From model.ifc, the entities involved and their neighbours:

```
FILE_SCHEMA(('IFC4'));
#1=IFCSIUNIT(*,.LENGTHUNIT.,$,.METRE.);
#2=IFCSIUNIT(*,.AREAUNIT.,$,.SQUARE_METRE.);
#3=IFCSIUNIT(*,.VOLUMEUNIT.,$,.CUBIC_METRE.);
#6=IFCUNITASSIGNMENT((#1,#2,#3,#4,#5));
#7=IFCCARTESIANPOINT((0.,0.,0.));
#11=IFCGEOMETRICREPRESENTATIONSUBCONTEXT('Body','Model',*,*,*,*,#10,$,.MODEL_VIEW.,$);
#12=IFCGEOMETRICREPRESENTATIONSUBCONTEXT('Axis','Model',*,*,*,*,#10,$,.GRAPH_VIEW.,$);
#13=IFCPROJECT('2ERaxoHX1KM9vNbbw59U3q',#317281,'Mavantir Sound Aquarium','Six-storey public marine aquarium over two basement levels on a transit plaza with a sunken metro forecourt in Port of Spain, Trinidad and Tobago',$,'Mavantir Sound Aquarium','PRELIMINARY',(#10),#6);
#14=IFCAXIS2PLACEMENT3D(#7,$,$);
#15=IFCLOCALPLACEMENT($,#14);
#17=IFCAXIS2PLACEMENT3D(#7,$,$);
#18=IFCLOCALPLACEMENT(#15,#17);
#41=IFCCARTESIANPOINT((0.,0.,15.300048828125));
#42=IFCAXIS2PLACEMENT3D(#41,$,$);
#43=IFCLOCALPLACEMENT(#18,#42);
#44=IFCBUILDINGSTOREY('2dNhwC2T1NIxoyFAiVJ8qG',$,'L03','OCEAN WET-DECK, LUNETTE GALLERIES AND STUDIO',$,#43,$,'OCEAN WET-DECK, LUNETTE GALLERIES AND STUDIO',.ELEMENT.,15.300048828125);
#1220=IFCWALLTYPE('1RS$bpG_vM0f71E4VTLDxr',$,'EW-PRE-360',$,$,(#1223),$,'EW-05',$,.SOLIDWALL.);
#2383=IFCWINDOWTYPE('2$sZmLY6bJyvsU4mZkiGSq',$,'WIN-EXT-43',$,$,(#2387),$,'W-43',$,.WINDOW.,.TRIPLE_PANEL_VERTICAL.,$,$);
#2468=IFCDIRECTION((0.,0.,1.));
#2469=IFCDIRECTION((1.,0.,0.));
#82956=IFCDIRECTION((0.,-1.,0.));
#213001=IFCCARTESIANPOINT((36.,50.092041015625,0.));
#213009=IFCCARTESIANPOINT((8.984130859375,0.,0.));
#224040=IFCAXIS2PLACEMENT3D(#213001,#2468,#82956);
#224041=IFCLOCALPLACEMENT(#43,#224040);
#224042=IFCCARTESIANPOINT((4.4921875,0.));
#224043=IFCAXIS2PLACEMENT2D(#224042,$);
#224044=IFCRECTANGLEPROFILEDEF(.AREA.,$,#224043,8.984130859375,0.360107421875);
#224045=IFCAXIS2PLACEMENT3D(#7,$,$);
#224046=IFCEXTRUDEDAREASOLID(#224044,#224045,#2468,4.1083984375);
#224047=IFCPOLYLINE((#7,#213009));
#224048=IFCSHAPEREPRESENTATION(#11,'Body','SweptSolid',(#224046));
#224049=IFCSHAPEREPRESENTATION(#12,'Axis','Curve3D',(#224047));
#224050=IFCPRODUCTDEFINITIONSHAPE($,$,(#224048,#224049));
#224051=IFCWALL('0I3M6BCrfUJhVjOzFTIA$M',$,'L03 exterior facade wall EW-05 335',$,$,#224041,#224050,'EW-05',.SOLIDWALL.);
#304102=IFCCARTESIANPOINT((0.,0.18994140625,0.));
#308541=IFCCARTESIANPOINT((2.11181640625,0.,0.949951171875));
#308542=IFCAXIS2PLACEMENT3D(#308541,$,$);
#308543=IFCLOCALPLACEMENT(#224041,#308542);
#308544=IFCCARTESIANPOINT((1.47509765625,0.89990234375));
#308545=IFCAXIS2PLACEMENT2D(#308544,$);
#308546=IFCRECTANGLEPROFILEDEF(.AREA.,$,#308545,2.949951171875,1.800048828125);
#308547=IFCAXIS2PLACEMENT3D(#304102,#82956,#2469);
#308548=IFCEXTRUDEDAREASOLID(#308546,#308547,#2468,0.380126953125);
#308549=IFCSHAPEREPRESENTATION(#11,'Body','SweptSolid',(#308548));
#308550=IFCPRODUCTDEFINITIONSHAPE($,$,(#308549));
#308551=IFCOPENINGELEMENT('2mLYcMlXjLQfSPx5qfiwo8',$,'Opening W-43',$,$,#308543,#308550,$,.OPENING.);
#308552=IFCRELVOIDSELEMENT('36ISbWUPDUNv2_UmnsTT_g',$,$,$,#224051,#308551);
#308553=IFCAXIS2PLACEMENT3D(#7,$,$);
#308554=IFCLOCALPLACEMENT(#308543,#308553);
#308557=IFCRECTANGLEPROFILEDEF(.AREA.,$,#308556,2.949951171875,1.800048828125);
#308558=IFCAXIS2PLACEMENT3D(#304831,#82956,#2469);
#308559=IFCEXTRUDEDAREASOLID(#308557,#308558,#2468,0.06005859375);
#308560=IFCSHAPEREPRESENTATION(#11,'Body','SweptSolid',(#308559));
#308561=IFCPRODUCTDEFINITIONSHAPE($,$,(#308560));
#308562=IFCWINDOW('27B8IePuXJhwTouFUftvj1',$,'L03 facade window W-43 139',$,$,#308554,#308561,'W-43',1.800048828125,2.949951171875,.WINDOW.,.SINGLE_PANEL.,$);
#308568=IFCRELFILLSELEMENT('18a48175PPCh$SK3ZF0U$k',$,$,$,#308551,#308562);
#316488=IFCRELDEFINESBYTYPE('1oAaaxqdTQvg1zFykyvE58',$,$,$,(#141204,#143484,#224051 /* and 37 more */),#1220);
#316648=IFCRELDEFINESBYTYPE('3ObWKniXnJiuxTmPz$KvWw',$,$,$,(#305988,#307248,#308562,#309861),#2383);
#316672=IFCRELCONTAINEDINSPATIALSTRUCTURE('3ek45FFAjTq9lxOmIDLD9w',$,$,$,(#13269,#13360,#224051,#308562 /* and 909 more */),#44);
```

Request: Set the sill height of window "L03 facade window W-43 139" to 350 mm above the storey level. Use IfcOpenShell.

```python
import numpy as np
import ifcopenshell
import ifcopenshell.api.geometry
import ifcopenshell.geom
import ifcopenshell.util.element
import ifcopenshell.util.placement
import ifcopenshell.util.shape
import ifcopenshell.util.unit

model = ifcopenshell.open("model.ifc")
unit_scale = ifcopenshell.util.unit.calculate_unit_scale(model)

window = model.by_guid("27B8IePuXJhwTouFUftvj1")
opening = window.FillsVoids[0].RelatingOpeningElement
storey = ifcopenshell.util.element.get_container(window, ifc_class="IfcBuildingStorey")
level = ifcopenshell.util.placement.get_local_placement(storey.ObjectPlacement)[2, 3]

# The opening's origin need not be at the sill, so measure its lowest point.
shape = ifcopenshell.geom.create_shape(ifcopenshell.geom.settings(), opening)
bottom = ifcopenshell.util.shape.get_shape_bottom_elevation(shape, shape.geometry) / unit_scale
dz = level + 0.35 - bottom

shift = np.array([0.0, 0.0, dz])
# The window is placed relative to its opening, so it follows when the opening moves.
matrix = ifcopenshell.util.placement.get_local_placement(opening.ObjectPlacement)
matrix[:3, 3] += shift
ifcopenshell.api.geometry.edit_object_placement(
    model, product=opening, matrix=matrix, is_si=False, should_transform_children=True
)

print(f"moved by {dz * unit_scale:+.3f} m")

model.write("model-out.ifc")
```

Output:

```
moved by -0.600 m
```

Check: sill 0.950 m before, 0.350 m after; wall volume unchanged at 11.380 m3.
